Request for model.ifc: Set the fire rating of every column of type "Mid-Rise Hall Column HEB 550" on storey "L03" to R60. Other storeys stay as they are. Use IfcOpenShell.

First a look at what the model holds.

```python
import ifcopenshell
import ifcopenshell.util.element

model = ifcopenshell.open("model.ifc")
print(model.schema)
storey = next(s for s in model.by_type("IfcBuildingStorey") if s.Name == "L03")
columns = [e for e in ifcopenshell.util.element.get_decomposition(storey) if e.is_a("IfcColumn")]
seen = {}
for e in columns:
    element_type = ifcopenshell.util.element.get_type(e)
    key = (element_type.Name if element_type != e and element_type else None, ifcopenshell.util.element.get_pset(e, "Pset_ColumnCommon", "FireRating"))
    seen[key] = seen.get(key, 0) + 1
for (name, value), count in sorted(seen.items(), key=str):
    print(count, "x", name, "|", value)
```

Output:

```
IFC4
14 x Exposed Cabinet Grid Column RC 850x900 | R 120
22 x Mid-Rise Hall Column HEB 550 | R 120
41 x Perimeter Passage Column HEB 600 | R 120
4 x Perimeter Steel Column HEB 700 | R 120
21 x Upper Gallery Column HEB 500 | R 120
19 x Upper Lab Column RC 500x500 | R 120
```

```python
import ifcopenshell
import ifcopenshell.api.pset
import ifcopenshell.util.element

model = ifcopenshell.open("model.ifc")

storey = next(s for s in model.by_type("IfcBuildingStorey") if s.Name == "L03")
columns = [e for e in ifcopenshell.util.element.get_decomposition(storey) if e.is_a("IfcColumn")]

count = 0
for e in columns:
    element_type = ifcopenshell.util.element.get_type(e)
    if element_type in (None, e) or element_type.Name != "Mid-Rise Hall Column HEB 550":
        continue
    # add_pset returns the element's existing set when there is one.
    pset = ifcopenshell.api.pset.add_pset(model, product=e, name="Pset_ColumnCommon")
    ifcopenshell.api.pset.edit_pset(model, pset=pset, properties={"FireRating": "R60"})
    count += 1

print(count, "columns updated")

model.write("model_updated.ifc")
```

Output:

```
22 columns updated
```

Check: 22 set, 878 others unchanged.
